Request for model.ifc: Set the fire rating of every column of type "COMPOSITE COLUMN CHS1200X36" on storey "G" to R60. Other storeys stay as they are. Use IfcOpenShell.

First a look at what the model holds.

```python
import ifcopenshell
import ifcopenshell.util.element

model = ifcopenshell.open("model.ifc")
print(model.schema)
storey = next(s for s in model.by_type("IfcBuildingStorey") if s.Name == "G")
columns = [e for e in ifcopenshell.util.element.get_decomposition(storey) if e.is_a("IfcColumn")]
seen = {}
for e in columns:
    element_type = ifcopenshell.util.element.get_type(e)
    key = (element_type.Name if element_type != e and element_type else None, ifcopenshell.util.element.get_pset(e, "Pset_ColumnCommon", "FireRating"))
    seen[key] = seen.get(key, 0) + 1
for (name, value), count in sorted(seen.items(), key=str):
    print(count, "x", name, "|", value)
```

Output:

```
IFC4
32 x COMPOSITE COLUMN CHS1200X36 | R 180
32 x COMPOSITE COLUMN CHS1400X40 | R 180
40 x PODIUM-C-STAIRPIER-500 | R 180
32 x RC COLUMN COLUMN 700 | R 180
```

```python
import ifcopenshell
import ifcopenshell.api.pset
import ifcopenshell.util.element

model = ifcopenshell.open("model.ifc")

storey = next(s for s in model.by_type("IfcBuildingStorey") if s.Name == "G")
columns = [e for e in ifcopenshell.util.element.get_decomposition(storey) if e.is_a("IfcColumn")]

count = 0
for e in columns:
    element_type = ifcopenshell.util.element.get_type(e)
    if element_type in (None, e) or element_type.Name != "COMPOSITE COLUMN CHS1200X36":
        continue
    found = ifcopenshell.util.element.get_pset(e, "Pset_ColumnCommon", should_inherit=False)
    if found:
        pset = model.by_id(found["id"])
        if len(ifcopenshell.util.element.get_elements_by_pset(pset)) > 1:
            pset = ifcopenshell.api.pset.unshare_pset(model, products=[e], pset=pset)[0]
    else:
        pset = ifcopenshell.api.pset.add_pset(model, product=e, name="Pset_ColumnCommon")
    ifcopenshell.api.pset.edit_pset(model, pset=pset, properties={"FireRating": "R60"})
    count += 1

print(count, "columns updated")

model.write("model_rev.ifc")
```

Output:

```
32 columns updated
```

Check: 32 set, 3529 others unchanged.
